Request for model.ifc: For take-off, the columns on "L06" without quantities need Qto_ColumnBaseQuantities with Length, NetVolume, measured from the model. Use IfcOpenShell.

First a look at what the model holds.

```python
import ifcopenshell
import ifcopenshell.util.element
import ifcopenshell.util.unit

model = ifcopenshell.open("model.ifc")
print(model.schema)
for unit_type in ("LENGTHUNIT", "AREAUNIT", "VOLUMEUNIT"):
    print(unit_type, ifcopenshell.util.unit.calculate_unit_scale(model, unit_type))
storey = next(s for s in model.by_type("IfcBuildingStorey") if s.Name == "L06")
columns = [e for e in ifcopenshell.util.element.get_decomposition(storey) if e.is_a("IfcColumn")]
for e in sorted(columns, key=lambda e: e.id()):
    print(e.id(), e.is_a(), e.Name, list(ifcopenshell.util.element.get_psets(e, qtos_only=True)), sep=" | ")
```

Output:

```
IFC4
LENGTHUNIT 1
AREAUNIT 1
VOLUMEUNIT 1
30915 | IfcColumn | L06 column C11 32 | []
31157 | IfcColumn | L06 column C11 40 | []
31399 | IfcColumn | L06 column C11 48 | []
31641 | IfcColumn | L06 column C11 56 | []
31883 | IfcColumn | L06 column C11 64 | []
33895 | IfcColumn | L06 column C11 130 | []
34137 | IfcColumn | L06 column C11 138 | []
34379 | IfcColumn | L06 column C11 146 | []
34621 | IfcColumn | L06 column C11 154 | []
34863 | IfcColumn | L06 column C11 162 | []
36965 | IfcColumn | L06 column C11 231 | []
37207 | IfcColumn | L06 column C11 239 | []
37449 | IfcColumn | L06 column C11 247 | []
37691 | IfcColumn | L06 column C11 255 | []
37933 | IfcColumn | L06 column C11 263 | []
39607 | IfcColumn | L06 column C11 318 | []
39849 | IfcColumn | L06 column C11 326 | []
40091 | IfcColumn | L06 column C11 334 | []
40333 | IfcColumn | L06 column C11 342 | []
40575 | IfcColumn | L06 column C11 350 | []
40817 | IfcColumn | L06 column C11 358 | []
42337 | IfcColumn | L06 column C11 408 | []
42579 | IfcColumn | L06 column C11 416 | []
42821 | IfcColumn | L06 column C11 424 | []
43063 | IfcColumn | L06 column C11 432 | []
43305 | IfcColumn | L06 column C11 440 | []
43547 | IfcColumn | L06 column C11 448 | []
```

```python
import ifcopenshell
import ifcopenshell.api.pset
import ifcopenshell.geom
import ifcopenshell.util.element
import ifcopenshell.util.shape
import ifcopenshell.util.unit

model = ifcopenshell.open("model.ifc")
unit_scale = ifcopenshell.util.unit.calculate_unit_scale(model)
volume_scale = ifcopenshell.util.unit.calculate_unit_scale(model, "VOLUMEUNIT")
settings = ifcopenshell.geom.settings()

storey = next(s for s in model.by_type("IfcBuildingStorey") if s.Name == "L06")
columns = [e for e in ifcopenshell.util.element.get_decomposition(storey) if e.is_a("IfcColumn")]

for e in sorted(columns, key=lambda e: e.id()):
    if ifcopenshell.util.element.get_psets(e, qtos_only=True, should_inherit=False):
        continue
    # Geometry comes back in metres, in the element's own axes.
    shape = ifcopenshell.geom.create_shape(settings, e)
    values = {
        "Length": ifcopenshell.util.shape.get_z(shape.geometry) / unit_scale,
        "NetVolume": ifcopenshell.util.shape.get_volume(shape.geometry) / volume_scale,
    }
    qto = ifcopenshell.api.pset.add_qto(model, product=e, name="Qto_ColumnBaseQuantities")
    ifcopenshell.api.pset.edit_qto(model, qto=qto, properties=values)
    print(e.id(), {k: round(v, 3) for k, v in values.items()})

model.write("model_updated.ifc")
```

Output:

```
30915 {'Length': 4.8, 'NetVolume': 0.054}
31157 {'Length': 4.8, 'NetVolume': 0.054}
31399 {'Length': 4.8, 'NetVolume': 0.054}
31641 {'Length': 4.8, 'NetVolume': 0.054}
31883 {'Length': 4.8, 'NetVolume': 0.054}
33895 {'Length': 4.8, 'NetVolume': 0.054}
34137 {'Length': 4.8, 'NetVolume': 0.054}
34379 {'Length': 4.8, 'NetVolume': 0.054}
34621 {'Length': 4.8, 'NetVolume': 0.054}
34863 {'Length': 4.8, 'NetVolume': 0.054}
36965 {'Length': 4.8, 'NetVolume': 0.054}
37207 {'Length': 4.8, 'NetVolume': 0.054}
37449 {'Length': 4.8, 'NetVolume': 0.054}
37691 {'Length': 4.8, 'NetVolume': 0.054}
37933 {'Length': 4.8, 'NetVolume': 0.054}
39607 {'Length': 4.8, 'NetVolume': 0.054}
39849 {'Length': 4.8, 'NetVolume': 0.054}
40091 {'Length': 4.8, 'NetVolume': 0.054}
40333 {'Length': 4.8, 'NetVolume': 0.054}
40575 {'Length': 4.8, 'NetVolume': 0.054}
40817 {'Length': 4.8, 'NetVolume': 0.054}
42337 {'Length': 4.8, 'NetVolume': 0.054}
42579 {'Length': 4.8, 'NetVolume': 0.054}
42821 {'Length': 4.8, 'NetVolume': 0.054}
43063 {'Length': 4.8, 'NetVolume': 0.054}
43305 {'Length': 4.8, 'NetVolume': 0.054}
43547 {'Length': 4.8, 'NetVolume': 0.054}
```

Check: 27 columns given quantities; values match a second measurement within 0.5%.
